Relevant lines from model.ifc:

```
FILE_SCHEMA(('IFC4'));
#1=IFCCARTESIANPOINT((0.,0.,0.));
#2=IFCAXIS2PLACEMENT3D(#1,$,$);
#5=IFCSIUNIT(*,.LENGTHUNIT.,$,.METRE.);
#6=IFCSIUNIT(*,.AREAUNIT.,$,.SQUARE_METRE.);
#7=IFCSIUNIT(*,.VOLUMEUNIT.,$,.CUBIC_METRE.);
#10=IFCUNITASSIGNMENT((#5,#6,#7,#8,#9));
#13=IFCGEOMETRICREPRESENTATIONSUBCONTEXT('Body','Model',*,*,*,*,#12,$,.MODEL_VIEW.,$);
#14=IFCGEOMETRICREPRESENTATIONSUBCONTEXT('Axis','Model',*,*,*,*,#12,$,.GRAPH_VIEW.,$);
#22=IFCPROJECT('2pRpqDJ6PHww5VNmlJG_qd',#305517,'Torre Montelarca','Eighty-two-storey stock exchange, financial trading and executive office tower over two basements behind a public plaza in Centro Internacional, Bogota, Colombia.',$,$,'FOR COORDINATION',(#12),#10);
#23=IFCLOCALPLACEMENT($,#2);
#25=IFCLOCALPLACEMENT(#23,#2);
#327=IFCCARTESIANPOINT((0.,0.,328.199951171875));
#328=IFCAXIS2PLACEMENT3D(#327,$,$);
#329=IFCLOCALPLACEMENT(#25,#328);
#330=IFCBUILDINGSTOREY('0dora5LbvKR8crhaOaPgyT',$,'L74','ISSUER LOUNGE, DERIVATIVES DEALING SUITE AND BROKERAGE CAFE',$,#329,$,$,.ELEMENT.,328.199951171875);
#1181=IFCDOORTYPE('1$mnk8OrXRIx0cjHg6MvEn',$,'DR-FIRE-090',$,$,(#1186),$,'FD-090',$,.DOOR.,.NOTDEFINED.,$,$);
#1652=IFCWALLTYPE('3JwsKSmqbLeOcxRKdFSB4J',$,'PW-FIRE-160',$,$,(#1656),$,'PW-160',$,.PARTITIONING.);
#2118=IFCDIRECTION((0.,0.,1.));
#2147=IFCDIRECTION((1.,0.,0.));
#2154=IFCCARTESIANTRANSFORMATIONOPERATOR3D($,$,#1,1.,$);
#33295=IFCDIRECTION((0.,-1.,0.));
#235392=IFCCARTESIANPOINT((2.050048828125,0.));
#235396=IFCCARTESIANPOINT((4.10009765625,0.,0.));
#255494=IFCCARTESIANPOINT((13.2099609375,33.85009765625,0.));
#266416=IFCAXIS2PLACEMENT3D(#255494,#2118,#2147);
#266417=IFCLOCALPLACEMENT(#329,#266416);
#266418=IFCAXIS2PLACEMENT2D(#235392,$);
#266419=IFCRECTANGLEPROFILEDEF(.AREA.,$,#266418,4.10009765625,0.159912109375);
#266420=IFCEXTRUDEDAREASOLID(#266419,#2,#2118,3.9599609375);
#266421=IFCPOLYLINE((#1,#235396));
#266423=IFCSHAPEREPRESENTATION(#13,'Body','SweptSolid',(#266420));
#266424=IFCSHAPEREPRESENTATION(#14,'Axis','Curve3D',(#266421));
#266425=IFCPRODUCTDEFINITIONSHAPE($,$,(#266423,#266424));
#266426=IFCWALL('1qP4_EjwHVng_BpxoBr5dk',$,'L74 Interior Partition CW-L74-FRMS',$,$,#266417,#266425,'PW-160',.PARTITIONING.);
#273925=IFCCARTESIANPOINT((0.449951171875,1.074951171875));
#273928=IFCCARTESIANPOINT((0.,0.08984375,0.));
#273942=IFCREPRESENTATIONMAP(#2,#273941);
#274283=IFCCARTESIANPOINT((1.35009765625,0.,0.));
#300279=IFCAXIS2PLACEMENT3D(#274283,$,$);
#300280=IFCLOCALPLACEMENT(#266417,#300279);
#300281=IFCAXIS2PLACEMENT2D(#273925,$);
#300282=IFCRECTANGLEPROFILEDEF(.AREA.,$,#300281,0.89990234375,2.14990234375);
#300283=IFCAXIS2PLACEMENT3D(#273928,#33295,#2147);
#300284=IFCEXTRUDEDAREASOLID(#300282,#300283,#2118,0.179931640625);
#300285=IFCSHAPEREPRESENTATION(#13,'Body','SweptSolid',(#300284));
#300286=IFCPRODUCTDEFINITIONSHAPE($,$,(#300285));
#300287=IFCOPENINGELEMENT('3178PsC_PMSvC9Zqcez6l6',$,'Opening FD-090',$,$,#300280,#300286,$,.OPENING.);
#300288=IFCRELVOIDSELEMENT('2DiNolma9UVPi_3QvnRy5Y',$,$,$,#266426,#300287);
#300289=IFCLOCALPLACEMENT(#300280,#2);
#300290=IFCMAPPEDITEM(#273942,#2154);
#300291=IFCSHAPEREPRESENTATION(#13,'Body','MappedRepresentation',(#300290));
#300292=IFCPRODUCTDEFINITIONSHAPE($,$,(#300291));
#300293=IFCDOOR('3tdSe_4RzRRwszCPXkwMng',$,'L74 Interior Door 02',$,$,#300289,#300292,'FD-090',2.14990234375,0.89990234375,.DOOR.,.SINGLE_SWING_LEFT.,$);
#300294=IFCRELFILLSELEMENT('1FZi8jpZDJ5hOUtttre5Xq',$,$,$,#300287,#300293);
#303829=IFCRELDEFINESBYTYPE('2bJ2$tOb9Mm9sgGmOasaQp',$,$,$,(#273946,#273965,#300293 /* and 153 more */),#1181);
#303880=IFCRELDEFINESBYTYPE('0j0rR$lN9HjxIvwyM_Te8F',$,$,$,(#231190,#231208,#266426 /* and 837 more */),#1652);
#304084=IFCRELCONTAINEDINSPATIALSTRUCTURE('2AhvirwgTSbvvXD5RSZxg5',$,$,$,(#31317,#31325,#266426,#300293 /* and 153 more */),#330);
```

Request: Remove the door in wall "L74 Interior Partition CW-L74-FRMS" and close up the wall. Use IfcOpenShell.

```python
import ifcopenshell
import ifcopenshell.api.feature
import ifcopenshell.api.root
import ifcopenshell.geom
import ifcopenshell.util.shape

model = ifcopenshell.open("model.ifc")
settings = ifcopenshell.geom.settings()


def volume(element):
    """Net volume in cubic metres, openings subtracted."""
    shape = ifcopenshell.geom.create_shape(settings, element)
    return ifcopenshell.util.shape.get_volume(shape.geometry)


door = model.by_id(300293)
opening = door.FillsVoids[0].RelatingOpeningElement
wall = opening.VoidsElements[0].RelatingBuildingElement
before = volume(wall)

ifcopenshell.api.root.remove_product(model, product=door)
ifcopenshell.api.feature.remove_feature(model, feature=opening)

after = volume(wall)

print(f"wall volume {before:.3f} -> {after:.3f} m3")

model.write("model-out.ifc")
```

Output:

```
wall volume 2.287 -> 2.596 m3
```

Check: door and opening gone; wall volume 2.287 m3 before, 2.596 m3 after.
